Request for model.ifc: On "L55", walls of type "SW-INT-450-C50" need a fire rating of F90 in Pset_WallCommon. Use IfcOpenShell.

First a look at what the model holds.

```python
import ifcopenshell
import ifcopenshell.util.element

model = ifcopenshell.open("model.ifc")
print(model.schema)
storey = next(s for s in model.by_type("IfcBuildingStorey") if s.Name == "L55")
walls = [e for e in ifcopenshell.util.element.get_decomposition(storey) if e.is_a("IfcWall")]
seen = {}
for e in walls:
    element_type = ifcopenshell.util.element.get_type(e)
    key = (element_type.Name if element_type != e and element_type else None, ifcopenshell.util.element.get_pset(e, "Pset_WallCommon", "FireRating"))
    seen[key] = seen.get(key, 0) + 1
for (name, value), count in sorted(seen.items(), key=str):
    print(count, "x", name, "|", value)
```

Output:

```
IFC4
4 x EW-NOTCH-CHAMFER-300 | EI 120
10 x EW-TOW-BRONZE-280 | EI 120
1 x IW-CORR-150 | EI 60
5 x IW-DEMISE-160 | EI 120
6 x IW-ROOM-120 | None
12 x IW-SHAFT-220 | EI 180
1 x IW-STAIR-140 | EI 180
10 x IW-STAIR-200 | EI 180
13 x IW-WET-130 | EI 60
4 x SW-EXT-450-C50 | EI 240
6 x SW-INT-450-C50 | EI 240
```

```python
import ifcopenshell
import ifcopenshell.api.pset
import ifcopenshell.util.element

model = ifcopenshell.open("model.ifc")

storey = next(s for s in model.by_type("IfcBuildingStorey") if s.Name == "L55")
walls = [e for e in ifcopenshell.util.element.get_decomposition(storey) if e.is_a("IfcWall")]

count = 0
for e in walls:
    element_type = ifcopenshell.util.element.get_type(e)
    if element_type in (None, e) or element_type.Name != "SW-INT-450-C50":
        continue
    found = ifcopenshell.util.element.get_pset(e, "Pset_WallCommon", should_inherit=False)
    if found:
        pset = model.by_id(found["id"])
        if len(ifcopenshell.util.element.get_elements_by_pset(pset)) > 1:
            pset = ifcopenshell.api.pset.unshare_pset(model, products=[e], pset=pset)[0]
    else:
        pset = ifcopenshell.api.pset.add_pset(model, product=e, name="Pset_WallCommon")
    ifcopenshell.api.pset.edit_pset(model, pset=pset, properties={"FireRating": "F90"})
    count += 1

print(count, "walls updated")

model.write("model_updated.ifc")
```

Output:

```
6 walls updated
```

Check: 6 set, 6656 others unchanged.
